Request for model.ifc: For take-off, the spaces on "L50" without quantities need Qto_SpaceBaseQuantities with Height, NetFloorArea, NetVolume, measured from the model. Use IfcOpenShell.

First a look at what the model holds.

```python
import ifcopenshell
import ifcopenshell.util.element
import ifcopenshell.util.unit

model = ifcopenshell.open("model.ifc")
print(model.schema)
for unit_type in ("LENGTHUNIT", "AREAUNIT", "VOLUMEUNIT"):
    print(unit_type, ifcopenshell.util.unit.calculate_unit_scale(model, unit_type))
storey = next(s for s in model.by_type("IfcBuildingStorey") if s.Name == "L50")
spaces = [e for e in ifcopenshell.util.element.get_decomposition(storey) if e.is_a("IfcSpace")]
for e in sorted(spaces, key=lambda e: e.id()):
    print(e.id(), e.is_a(), e.Name, list(ifcopenshell.util.element.get_psets(e, qtos_only=True)), sep=" | ")
```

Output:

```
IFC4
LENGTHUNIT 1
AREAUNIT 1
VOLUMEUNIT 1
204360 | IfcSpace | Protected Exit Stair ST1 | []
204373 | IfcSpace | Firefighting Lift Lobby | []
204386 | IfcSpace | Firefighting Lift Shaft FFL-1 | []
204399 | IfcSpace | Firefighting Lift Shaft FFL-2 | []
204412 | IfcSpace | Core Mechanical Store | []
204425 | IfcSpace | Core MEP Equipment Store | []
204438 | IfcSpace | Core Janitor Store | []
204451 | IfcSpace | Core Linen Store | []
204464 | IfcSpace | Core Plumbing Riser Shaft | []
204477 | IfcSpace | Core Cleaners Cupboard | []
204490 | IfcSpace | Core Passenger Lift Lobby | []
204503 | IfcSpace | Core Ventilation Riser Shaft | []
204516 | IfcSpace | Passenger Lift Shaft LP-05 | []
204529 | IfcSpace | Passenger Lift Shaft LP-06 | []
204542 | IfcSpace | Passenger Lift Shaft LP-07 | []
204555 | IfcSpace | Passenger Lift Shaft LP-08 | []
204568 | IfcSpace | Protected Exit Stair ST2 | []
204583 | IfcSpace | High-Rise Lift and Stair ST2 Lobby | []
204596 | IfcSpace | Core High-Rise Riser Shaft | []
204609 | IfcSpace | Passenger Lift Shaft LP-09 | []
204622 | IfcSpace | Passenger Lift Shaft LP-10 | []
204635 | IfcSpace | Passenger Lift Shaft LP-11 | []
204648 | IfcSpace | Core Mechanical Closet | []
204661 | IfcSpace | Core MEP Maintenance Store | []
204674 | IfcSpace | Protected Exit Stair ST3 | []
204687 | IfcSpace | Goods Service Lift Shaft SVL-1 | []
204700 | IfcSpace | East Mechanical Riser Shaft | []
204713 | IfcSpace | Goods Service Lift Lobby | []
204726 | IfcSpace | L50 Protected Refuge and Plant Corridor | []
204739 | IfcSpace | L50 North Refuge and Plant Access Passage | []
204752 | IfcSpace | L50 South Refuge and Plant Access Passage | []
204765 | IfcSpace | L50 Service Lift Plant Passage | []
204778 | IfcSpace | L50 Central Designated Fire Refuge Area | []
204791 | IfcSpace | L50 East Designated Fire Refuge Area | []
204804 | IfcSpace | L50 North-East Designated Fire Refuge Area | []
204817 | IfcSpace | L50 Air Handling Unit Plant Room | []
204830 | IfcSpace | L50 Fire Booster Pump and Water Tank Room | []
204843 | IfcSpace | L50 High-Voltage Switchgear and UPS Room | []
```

```python
import ifcopenshell
import ifcopenshell.api.pset
import ifcopenshell.geom
import ifcopenshell.util.element
import ifcopenshell.util.shape
import ifcopenshell.util.unit

model = ifcopenshell.open("model.ifc")
unit_scale = ifcopenshell.util.unit.calculate_unit_scale(model)
area_scale = ifcopenshell.util.unit.calculate_unit_scale(model, "AREAUNIT")
volume_scale = ifcopenshell.util.unit.calculate_unit_scale(model, "VOLUMEUNIT")
settings = ifcopenshell.geom.settings()

storey = next(s for s in model.by_type("IfcBuildingStorey") if s.Name == "L50")
spaces = [e for e in ifcopenshell.util.element.get_decomposition(storey) if e.is_a("IfcSpace")]

for e in sorted(spaces, key=lambda e: e.id()):
    if ifcopenshell.util.element.get_psets(e, qtos_only=True, should_inherit=False):
        continue
    # Geometry comes back in metres, in the element's own axes.
    shape = ifcopenshell.geom.create_shape(settings, e)
    values = {
        "Height": ifcopenshell.util.shape.get_z(shape.geometry) / unit_scale,
        "NetFloorArea": ifcopenshell.util.shape.get_footprint_area(shape.geometry) / area_scale,
        "NetVolume": ifcopenshell.util.shape.get_volume(shape.geometry) / volume_scale,
    }
    qto = ifcopenshell.api.pset.add_qto(model, product=e, name="Qto_SpaceBaseQuantities")
    ifcopenshell.api.pset.edit_qto(model, qto=qto, properties=values)
    print(e.id(), {k: round(v, 3) for k, v in values.items()})

model.write("model_rev.ifc")
```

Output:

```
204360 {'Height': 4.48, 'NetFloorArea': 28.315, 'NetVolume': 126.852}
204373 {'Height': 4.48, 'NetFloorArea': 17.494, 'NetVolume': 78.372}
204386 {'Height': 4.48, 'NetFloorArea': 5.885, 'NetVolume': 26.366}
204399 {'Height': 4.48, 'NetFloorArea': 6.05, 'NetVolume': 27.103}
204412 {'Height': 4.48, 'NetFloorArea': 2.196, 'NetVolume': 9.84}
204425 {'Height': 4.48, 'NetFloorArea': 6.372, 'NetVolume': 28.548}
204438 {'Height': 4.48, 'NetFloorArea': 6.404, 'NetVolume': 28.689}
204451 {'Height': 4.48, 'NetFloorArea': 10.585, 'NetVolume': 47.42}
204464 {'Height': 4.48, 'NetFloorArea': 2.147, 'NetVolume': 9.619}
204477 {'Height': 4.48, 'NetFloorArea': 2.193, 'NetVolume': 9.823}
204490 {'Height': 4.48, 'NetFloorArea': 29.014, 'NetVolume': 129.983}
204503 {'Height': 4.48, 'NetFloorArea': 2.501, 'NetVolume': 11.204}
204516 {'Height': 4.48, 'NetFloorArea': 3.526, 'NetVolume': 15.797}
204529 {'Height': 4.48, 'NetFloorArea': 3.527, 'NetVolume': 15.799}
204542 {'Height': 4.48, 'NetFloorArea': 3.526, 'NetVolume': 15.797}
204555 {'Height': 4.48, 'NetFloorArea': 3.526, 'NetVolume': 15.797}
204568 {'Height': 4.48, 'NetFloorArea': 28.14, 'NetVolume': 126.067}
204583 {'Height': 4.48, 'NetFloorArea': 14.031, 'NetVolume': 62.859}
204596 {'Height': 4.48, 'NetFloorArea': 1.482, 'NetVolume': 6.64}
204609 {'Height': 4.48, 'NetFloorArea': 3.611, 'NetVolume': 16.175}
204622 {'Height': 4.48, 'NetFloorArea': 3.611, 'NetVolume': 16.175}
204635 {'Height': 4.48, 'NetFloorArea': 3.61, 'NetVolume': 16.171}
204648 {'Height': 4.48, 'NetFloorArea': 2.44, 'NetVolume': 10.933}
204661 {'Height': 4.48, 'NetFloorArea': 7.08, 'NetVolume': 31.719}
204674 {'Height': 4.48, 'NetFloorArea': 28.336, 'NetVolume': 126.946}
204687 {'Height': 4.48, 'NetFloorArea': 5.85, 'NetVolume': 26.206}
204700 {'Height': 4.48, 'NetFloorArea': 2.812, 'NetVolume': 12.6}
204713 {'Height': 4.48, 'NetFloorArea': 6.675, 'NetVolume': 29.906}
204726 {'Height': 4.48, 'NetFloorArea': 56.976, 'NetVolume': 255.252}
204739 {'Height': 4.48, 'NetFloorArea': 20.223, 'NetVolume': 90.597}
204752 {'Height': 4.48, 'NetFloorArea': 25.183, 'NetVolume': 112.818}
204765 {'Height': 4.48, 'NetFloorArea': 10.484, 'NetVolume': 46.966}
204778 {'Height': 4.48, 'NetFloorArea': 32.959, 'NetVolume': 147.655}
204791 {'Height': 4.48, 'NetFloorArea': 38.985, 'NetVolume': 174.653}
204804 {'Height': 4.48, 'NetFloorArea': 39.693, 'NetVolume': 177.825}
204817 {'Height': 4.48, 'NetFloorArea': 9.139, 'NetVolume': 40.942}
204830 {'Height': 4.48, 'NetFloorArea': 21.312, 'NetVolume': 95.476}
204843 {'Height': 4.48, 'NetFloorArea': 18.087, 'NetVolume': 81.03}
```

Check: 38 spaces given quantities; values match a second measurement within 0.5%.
